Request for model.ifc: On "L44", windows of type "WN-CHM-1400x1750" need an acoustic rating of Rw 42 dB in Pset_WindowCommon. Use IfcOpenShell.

First a look at what the model holds.

```python
import ifcopenshell
import ifcopenshell.util.element

model = ifcopenshell.open("model.ifc")
print(model.schema)
storey = next(s for s in model.by_type("IfcBuildingStorey") if s.Name == "L44")
windows = [e for e in ifcopenshell.util.element.get_decomposition(storey) if e.is_a("IfcWindow")]
seen = {}
for e in windows:
    element_type = ifcopenshell.util.element.get_type(e)
    key = (element_type.Name if element_type != e and element_type else None, ifcopenshell.util.element.get_pset(e, "Pset_WindowCommon", "AcousticRating"))
    seen[key] = seen.get(key, 0) + 1
for (name, value), count in sorted(seen.items(), key=str):
    print(count, "x", name, "|", value)
```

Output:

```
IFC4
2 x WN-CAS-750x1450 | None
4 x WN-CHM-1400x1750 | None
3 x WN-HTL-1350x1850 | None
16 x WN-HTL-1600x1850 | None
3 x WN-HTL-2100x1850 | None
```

```python
import ifcopenshell
import ifcopenshell.api.pset
import ifcopenshell.util.element

model = ifcopenshell.open("model.ifc")

storey = next(s for s in model.by_type("IfcBuildingStorey") if s.Name == "L44")
windows = [e for e in ifcopenshell.util.element.get_decomposition(storey) if e.is_a("IfcWindow")]

count = 0
for e in windows:
    element_type = ifcopenshell.util.element.get_type(e)
    if element_type in (None, e) or element_type.Name != "WN-CHM-1400x1750":
        continue
    # add_pset returns the element's existing set when there is one.
    pset = ifcopenshell.api.pset.add_pset(model, product=e, name="Pset_WindowCommon")
    ifcopenshell.api.pset.edit_pset(model, pset=pset, properties={"AcousticRating": "Rw 42 dB"})
    count += 1

print(count, "windows updated")

model.write("model_updated.ifc")
```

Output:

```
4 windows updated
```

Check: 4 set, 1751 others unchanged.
